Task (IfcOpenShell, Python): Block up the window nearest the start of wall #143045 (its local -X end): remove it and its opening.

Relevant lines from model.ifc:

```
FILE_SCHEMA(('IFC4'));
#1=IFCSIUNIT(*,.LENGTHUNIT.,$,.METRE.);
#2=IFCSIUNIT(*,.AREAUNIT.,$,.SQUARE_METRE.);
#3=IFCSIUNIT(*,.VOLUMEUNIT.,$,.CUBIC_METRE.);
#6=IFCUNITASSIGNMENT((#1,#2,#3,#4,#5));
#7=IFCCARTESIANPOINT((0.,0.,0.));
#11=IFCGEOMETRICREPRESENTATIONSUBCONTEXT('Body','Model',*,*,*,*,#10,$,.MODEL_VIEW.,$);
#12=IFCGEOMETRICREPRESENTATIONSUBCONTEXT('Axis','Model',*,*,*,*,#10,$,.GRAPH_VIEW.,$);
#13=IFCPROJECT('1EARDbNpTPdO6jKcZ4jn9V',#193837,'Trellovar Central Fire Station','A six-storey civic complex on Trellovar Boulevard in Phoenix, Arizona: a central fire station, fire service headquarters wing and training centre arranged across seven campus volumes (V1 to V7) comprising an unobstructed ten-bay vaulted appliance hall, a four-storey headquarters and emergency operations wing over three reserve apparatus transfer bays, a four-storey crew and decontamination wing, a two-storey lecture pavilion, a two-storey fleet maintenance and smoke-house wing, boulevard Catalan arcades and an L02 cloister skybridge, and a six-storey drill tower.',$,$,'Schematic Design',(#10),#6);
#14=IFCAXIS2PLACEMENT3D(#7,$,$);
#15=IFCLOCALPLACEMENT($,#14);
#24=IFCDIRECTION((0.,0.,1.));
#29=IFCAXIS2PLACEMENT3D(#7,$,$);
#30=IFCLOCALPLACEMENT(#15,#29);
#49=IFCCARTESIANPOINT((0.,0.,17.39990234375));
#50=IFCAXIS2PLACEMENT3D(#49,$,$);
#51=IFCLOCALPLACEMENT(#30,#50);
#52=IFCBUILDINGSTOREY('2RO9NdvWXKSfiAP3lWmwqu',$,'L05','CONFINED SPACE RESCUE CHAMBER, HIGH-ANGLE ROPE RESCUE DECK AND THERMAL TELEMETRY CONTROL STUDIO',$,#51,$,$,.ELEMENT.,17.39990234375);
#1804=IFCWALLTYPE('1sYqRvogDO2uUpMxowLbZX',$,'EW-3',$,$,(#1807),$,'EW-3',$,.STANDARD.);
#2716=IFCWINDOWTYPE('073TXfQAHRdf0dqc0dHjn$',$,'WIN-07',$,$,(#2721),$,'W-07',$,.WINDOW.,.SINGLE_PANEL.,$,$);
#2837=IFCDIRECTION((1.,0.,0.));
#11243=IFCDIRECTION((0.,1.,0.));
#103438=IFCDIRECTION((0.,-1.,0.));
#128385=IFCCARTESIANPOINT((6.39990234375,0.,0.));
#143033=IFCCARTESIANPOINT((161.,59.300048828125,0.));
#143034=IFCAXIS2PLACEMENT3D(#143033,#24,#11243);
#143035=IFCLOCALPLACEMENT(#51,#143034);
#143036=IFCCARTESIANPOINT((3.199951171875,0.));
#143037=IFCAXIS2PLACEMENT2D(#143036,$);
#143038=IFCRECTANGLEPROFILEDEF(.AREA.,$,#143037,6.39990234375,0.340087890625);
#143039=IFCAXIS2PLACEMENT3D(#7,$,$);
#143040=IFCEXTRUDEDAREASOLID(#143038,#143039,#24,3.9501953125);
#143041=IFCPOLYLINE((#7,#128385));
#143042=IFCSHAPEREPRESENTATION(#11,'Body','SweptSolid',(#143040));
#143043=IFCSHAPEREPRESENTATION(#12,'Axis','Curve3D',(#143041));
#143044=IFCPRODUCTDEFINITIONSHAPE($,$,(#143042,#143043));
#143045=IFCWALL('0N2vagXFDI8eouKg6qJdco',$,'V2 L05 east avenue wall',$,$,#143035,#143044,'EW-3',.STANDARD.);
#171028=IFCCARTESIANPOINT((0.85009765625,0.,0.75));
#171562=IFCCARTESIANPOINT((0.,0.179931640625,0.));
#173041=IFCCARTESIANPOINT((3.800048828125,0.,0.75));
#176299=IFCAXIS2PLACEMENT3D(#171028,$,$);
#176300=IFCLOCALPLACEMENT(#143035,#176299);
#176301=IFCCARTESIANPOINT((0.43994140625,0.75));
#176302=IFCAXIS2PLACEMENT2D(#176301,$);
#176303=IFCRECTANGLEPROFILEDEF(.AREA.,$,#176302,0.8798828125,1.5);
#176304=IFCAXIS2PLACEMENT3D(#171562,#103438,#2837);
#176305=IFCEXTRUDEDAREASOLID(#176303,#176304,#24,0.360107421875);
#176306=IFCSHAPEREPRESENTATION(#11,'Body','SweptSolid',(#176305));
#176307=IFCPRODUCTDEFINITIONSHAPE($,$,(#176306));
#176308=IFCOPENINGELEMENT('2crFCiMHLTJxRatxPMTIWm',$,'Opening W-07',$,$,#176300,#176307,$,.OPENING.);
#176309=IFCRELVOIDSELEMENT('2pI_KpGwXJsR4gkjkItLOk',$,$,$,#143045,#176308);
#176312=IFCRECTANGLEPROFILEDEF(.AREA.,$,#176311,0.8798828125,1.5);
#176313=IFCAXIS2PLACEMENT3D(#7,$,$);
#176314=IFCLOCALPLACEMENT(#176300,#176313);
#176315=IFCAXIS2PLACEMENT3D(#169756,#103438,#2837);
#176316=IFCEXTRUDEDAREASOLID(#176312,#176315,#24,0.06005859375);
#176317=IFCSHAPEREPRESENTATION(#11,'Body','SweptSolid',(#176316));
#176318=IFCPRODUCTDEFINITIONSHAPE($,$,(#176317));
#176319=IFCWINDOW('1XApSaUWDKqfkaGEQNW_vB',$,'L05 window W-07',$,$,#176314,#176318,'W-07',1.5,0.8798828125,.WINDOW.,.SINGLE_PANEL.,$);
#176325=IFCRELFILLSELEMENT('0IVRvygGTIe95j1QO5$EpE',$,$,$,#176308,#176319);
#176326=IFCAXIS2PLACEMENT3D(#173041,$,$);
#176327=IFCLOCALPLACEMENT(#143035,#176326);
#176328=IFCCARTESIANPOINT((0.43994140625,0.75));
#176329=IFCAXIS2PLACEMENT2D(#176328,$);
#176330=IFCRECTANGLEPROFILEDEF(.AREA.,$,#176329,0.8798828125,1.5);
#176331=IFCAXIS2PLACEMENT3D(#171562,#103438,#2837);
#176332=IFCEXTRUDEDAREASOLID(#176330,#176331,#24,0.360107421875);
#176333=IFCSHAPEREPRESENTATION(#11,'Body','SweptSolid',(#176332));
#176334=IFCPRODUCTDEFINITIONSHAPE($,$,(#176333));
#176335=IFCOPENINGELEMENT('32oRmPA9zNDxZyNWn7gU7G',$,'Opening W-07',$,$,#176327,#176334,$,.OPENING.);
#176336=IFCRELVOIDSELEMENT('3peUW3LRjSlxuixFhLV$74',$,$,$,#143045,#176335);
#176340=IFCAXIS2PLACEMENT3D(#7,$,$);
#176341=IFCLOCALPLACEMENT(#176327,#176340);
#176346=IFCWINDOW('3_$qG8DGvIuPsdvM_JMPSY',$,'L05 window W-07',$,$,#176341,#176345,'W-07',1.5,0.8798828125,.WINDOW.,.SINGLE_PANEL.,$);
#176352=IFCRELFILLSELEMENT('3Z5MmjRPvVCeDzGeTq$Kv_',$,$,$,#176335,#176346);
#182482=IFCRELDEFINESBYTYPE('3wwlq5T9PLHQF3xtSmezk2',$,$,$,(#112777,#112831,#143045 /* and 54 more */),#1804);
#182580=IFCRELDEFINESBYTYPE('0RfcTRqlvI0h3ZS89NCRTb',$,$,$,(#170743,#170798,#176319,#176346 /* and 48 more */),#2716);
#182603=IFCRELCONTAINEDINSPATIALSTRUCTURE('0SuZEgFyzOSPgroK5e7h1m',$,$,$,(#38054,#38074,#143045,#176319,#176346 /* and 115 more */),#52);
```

```python
import ifcopenshell
import ifcopenshell.api.feature
import ifcopenshell.api.root
import ifcopenshell.geom
import ifcopenshell.util.shape

model = ifcopenshell.open("model.ifc")
settings = ifcopenshell.geom.settings()


def volume(element):
    """Net volume in cubic metres, openings subtracted."""
    shape = ifcopenshell.geom.create_shape(settings, element)
    return ifcopenshell.util.shape.get_volume(shape.geometry)


window = model.by_guid("1XApSaUWDKqfkaGEQNW_vB")
opening = window.FillsVoids[0].RelatingOpeningElement
wall = opening.VoidsElements[0].RelatingBuildingElement
before = volume(wall)

ifcopenshell.api.root.remove_product(model, product=window)
ifcopenshell.api.feature.remove_feature(model, feature=opening)

after = volume(wall)

print(f"wall volume {before:.3f} -> {after:.3f} m3")

model.write("model_edited.ifc")
```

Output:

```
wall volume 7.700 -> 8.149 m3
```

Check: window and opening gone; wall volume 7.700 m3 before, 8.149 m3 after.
